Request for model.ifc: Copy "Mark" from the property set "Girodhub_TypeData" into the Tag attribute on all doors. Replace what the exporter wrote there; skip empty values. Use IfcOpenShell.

First a look at what the model holds.

```python
import ifcopenshell
import ifcopenshell.util.element

model = ifcopenshell.open("model.ifc")
print(model.schema)
doors = model.by_type("IfcDoor")
print(len(doors), "doors")
for e in doors[:8]:
    source = ifcopenshell.util.element.get_pset(e, "Girodhub_TypeData", "Mark")
    target = e.Tag
    print(e.id(), repr(source), repr(target), sep=" | ")
```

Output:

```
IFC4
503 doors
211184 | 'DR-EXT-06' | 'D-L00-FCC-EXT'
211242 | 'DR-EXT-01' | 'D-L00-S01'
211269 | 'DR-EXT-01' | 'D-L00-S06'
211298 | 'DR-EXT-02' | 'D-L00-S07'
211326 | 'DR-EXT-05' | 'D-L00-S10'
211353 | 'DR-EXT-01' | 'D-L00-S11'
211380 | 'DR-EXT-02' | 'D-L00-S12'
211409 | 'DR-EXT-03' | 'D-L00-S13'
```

```python
import ifcopenshell
import ifcopenshell.util.element

model = ifcopenshell.open("model.ifc")

count = 0
for e in model.by_type("IfcDoor"):
    value = ifcopenshell.util.element.get_pset(e, "Girodhub_TypeData", "Mark")
    current = e.Tag
    if not value or not value.strip() or current == value:
        continue
    e.Tag = value
    count += 1

print(count, "doors updated")

model.write("model-out.ifc")
```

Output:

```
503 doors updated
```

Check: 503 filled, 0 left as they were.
